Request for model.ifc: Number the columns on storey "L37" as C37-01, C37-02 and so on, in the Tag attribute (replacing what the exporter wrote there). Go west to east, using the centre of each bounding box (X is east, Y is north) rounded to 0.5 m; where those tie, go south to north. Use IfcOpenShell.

First a look at what the model holds.

```python
import ifcopenshell
import ifcopenshell.util.element
import ifcopenshell.util.placement

model = ifcopenshell.open("model.ifc")
print(model.schema)
storey = next(s for s in model.by_type("IfcBuildingStorey") if s.Name == "L37")
columns = [e for e in ifcopenshell.util.element.get_decomposition(storey) if e.is_a("IfcColumn")]
for e in sorted(columns, key=lambda e: e.id()):
    origin = ifcopenshell.util.placement.get_local_placement(e.ObjectPlacement)[:3, 3]
    print(e.id(), e.Tag, e.Name, origin.round(2) + 0.0, sep=" | ")
```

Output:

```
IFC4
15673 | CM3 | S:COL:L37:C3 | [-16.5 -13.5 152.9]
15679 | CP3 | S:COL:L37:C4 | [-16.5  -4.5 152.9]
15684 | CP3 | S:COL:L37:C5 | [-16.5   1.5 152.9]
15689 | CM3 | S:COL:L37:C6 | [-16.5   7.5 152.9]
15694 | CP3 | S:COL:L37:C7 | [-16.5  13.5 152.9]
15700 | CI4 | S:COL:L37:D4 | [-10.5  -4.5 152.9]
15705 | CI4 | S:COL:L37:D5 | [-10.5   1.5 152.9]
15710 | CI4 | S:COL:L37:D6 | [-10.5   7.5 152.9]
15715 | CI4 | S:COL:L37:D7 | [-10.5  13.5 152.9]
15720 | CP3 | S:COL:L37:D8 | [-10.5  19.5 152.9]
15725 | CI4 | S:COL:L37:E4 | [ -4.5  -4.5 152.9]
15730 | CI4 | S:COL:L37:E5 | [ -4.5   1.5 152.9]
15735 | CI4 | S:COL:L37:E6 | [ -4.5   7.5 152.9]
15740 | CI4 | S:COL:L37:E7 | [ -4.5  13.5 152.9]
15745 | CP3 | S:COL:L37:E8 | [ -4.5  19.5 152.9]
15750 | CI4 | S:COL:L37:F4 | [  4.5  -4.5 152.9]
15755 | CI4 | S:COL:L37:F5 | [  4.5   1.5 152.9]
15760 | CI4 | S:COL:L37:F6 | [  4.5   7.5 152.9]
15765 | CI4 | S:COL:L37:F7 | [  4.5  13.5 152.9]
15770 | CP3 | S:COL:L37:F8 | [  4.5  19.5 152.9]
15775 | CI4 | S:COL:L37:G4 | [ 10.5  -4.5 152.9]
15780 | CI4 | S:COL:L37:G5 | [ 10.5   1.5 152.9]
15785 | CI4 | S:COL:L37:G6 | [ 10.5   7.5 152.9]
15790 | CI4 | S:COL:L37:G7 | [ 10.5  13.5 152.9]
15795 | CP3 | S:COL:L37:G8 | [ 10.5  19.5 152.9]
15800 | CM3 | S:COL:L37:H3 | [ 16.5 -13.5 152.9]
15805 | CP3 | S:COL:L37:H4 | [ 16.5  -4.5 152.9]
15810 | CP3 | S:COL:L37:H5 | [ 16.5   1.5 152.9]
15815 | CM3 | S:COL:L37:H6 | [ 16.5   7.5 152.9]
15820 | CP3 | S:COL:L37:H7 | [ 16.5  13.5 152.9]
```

```python
import ifcopenshell
import ifcopenshell.geom
import ifcopenshell.util.element
import ifcopenshell.util.shape

model = ifcopenshell.open("model.ifc")
settings = ifcopenshell.geom.settings()
settings.set("use-world-coords", True)


def centre(element):
    shape = ifcopenshell.geom.create_shape(settings, element)
    return ifcopenshell.util.shape.get_bbox_centroid(shape.geometry)


storey = next(s for s in model.by_type("IfcBuildingStorey") if s.Name == "L37")
columns = [e for e in ifcopenshell.util.element.get_decomposition(storey) if e.is_a("IfcColumn")]

# Insertion points can sit at a corner or the storey origin, so sort by the geometry (in metres).
centres = {e: centre(e) for e in columns}
columns.sort(key=lambda e: (round(centres[e][0] / 0.5), centres[e][1]))

for i, e in enumerate(columns, start=1):
    number = f"C37-{i:02d}"
    e.Tag = number
    print(e.id(), number)

model.write("model-out.ifc")
```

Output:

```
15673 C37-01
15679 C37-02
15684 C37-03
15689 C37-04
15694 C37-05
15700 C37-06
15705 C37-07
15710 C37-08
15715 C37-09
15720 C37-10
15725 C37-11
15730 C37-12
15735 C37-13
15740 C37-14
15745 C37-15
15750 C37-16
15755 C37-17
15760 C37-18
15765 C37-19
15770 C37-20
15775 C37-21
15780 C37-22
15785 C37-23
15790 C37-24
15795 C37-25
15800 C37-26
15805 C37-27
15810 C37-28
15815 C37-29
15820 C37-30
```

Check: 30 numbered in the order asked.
